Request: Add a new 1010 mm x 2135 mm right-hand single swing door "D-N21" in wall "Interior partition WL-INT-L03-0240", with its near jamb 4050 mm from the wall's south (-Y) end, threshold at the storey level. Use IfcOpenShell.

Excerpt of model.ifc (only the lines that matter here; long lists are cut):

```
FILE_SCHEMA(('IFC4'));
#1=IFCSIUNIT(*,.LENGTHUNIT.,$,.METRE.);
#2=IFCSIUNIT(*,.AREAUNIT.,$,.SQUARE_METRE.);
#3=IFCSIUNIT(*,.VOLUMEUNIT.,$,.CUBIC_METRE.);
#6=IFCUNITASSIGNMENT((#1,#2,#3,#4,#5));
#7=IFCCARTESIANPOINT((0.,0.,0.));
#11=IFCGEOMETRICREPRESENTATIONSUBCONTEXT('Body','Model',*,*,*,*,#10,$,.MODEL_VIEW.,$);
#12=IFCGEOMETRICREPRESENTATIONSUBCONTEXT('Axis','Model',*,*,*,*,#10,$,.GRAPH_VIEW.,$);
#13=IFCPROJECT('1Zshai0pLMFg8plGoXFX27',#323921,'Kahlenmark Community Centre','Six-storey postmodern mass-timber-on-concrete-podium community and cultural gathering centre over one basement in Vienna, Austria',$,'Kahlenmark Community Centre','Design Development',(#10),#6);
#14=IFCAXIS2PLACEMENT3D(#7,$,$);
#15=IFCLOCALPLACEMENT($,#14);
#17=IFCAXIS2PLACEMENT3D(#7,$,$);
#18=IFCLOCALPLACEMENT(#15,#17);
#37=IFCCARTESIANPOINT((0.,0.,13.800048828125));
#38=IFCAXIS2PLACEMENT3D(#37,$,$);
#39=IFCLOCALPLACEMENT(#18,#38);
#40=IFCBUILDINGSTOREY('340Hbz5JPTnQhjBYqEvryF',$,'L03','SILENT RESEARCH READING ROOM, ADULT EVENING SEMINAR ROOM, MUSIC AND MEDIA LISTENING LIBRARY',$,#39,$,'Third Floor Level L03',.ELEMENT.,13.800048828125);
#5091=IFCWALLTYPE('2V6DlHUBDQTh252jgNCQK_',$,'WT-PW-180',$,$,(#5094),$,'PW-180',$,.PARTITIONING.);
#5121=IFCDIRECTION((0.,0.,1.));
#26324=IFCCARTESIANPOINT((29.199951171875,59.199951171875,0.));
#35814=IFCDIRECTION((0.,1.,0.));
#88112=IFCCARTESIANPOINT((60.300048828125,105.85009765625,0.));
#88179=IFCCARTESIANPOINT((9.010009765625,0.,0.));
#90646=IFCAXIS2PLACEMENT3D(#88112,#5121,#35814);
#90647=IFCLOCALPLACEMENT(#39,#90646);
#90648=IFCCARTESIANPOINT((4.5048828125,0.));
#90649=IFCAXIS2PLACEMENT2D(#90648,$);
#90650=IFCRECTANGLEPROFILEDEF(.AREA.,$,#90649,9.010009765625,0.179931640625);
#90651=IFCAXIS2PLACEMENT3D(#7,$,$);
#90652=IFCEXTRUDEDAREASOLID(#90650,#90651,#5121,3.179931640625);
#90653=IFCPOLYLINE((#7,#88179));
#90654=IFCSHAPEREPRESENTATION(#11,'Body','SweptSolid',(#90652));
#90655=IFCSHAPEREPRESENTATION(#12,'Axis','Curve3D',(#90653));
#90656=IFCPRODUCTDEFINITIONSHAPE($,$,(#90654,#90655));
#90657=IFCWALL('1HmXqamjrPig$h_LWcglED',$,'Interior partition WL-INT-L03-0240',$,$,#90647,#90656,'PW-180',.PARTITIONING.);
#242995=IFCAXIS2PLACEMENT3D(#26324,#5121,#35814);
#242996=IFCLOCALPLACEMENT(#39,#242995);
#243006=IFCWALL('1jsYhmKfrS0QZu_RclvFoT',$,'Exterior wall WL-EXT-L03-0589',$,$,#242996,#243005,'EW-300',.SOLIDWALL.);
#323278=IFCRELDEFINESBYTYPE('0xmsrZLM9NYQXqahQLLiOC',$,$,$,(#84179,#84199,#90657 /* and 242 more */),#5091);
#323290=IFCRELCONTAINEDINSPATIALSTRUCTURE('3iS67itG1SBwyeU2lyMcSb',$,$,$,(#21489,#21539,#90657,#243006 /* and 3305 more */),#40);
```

```python
import numpy as np
import ifcopenshell
import ifcopenshell.api.feature
import ifcopenshell.api.geometry
import ifcopenshell.api.root
import ifcopenshell.api.spatial
import ifcopenshell.geom
import ifcopenshell.util.element
import ifcopenshell.util.placement
import ifcopenshell.util.representation
import ifcopenshell.util.shape
import ifcopenshell.util.unit

model = ifcopenshell.open("model.ifc")
unit_scale = ifcopenshell.util.unit.calculate_unit_scale(model)
settings = ifcopenshell.geom.settings()


def volume(element):
    """Net volume in cubic metres, openings subtracted."""
    shape = ifcopenshell.geom.create_shape(settings, element)
    return ifcopenshell.util.shape.get_volume(shape.geometry)


wall = model.by_id(90657)
storey = ifcopenshell.util.element.get_container(wall, ifc_class="IfcBuildingStorey")
context = ifcopenshell.util.representation.get_context(model, "Model", "Body", "MODEL_VIEW")
before = volume(wall)

width, height, from_end, sill = 1.01, 2.135, 4.05, 0.0  # metres

# The wall runs along its own X axis, and the end named is its -X end.
wall_shape = ifcopenshell.geom.create_shape(settings, wall)
x, y, z = ifcopenshell.util.shape.get_vertices(wall_shape.geometry).T
start = x.min() + from_end
face, thickness = float(y.min()), float(y.max() - y.min())
wall_matrix = ifcopenshell.util.placement.get_local_placement(wall.ObjectPlacement)
level = ifcopenshell.util.placement.get_local_placement(storey.ObjectPlacement)[2, 3]


def in_wall(x, y):
    """Placement at x, y metres in the wall's axes, at sill height."""
    matrix = wall_matrix.copy()
    matrix[:, 3] = wall_matrix @ np.array([x / unit_scale, y / unit_scale, 0.0, 1.0])
    matrix[2, 3] = level + sill / unit_scale
    return matrix


# Opening: a box that overshoots both wall faces by 50 mm.
opening = ifcopenshell.api.root.create_entity(model, ifc_class="IfcOpeningElement", predefined_type="OPENING")
box = ifcopenshell.api.geometry.add_wall_representation(
    model, context=context, length=width, height=height, thickness=thickness + 0.1
)
ifcopenshell.api.geometry.assign_representation(model, product=opening, representation=box)
ifcopenshell.api.geometry.edit_object_placement(model, product=opening, matrix=in_wall(start, face - 0.05), is_si=False)
ifcopenshell.api.feature.add_feature(model, feature=opening, element=wall)

door = ifcopenshell.api.root.create_entity(model, ifc_class="IfcDoor", name="D-N21", predefined_type="DOOR")
door.OverallWidth, door.OverallHeight = width / unit_scale, height / unit_scale
door.OperationType = "SINGLE_SWING_RIGHT"
body = ifcopenshell.api.geometry.add_door_representation(
    model,
    context=context,
    overall_width=door.OverallWidth,
    overall_height=door.OverallHeight,
    operation_type="SINGLE_SWING_RIGHT",
    lining_properties={"LiningDepth": thickness / unit_scale, "ThresholdDepth": thickness / unit_scale},
)
ifcopenshell.api.geometry.assign_representation(model, product=door, representation=body)
ifcopenshell.api.spatial.assign_container(model, products=[door], relating_structure=storey)
ifcopenshell.api.feature.add_filling(model, opening=opening, element=door)

# The lining spans the wall, so the door starts at the wall face.
ifcopenshell.api.geometry.edit_object_placement(model, product=door, matrix=in_wall(start, face), is_si=False)

after = volume(wall)

print(f"wall volume {before:.3f} -> {after:.3f} m3")

model.write("model_rev.ifc")
```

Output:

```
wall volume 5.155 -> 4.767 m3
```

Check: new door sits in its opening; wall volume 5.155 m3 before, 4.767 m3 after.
